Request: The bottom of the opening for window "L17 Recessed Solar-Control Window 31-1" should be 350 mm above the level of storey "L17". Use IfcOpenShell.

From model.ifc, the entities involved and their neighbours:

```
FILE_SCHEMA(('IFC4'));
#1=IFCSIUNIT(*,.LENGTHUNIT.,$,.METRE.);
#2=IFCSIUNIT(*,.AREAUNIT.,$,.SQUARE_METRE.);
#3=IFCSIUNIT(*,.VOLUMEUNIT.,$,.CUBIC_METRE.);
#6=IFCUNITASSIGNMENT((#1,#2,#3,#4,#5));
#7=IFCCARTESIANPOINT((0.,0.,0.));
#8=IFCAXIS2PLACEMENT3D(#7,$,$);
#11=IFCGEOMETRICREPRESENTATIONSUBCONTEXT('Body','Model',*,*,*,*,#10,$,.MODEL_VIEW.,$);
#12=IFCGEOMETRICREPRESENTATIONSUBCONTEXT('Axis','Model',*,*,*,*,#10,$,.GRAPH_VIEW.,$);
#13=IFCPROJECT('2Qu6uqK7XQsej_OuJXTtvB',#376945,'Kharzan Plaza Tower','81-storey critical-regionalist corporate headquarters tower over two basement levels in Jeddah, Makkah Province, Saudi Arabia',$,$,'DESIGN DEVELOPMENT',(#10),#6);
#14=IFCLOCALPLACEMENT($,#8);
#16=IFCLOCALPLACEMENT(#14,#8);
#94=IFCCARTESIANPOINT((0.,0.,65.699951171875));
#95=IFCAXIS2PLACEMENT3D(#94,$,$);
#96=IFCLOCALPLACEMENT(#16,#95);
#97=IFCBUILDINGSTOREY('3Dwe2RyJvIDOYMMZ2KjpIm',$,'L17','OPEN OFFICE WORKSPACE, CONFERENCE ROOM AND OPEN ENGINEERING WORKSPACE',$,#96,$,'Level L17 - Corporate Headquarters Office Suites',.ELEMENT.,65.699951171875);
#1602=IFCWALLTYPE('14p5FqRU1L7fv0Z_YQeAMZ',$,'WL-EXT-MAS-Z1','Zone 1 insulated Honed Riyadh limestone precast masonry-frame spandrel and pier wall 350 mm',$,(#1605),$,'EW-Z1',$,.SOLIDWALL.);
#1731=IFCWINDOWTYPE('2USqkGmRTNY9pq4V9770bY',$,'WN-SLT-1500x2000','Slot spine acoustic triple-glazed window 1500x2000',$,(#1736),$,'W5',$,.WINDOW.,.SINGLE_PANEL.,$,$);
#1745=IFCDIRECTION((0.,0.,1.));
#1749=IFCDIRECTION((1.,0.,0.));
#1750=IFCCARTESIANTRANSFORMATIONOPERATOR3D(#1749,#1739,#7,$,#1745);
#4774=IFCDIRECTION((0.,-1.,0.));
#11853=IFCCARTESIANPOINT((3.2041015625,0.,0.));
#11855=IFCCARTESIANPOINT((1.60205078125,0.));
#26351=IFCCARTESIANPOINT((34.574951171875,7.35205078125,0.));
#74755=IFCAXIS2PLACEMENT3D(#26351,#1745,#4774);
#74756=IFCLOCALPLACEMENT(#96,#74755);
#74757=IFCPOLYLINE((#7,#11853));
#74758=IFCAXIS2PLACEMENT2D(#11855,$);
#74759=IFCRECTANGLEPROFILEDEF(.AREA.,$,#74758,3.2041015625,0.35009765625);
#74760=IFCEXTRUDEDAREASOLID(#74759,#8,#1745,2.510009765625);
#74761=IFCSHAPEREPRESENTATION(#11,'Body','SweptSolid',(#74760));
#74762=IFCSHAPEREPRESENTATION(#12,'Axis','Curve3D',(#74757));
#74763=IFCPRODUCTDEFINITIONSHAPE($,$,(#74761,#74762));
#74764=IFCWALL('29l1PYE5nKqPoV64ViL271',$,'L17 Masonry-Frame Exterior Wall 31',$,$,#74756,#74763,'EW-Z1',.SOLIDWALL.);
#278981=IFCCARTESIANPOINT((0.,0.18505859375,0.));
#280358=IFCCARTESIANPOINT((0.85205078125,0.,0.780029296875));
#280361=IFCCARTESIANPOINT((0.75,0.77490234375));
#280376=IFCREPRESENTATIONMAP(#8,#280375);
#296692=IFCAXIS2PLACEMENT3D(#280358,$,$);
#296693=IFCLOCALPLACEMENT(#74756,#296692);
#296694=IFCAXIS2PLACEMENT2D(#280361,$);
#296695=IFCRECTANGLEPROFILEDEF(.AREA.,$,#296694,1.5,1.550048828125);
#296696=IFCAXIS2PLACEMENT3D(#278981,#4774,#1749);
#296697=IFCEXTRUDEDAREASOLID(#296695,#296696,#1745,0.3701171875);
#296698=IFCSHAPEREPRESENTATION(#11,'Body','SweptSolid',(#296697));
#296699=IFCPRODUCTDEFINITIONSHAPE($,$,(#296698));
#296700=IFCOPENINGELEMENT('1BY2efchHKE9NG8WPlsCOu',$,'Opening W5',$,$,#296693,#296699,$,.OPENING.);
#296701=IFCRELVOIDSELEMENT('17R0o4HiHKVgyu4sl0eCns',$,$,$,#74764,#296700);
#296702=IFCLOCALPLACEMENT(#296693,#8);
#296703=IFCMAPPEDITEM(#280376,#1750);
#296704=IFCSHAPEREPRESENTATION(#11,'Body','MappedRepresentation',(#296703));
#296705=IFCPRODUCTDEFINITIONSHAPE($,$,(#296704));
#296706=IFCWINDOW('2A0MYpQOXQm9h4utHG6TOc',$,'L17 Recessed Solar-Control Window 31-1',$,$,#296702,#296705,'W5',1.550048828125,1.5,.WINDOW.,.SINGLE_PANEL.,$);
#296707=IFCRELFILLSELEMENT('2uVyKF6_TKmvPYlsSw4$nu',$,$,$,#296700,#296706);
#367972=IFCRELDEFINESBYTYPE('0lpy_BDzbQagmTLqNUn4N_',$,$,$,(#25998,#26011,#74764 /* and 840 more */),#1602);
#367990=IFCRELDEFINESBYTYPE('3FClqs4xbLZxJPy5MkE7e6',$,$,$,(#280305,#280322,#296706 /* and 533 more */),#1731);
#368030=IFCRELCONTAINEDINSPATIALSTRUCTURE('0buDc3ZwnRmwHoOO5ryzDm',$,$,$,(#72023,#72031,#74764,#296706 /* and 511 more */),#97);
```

```python
import numpy as np
import ifcopenshell
import ifcopenshell.api.geometry
import ifcopenshell.geom
import ifcopenshell.util.element
import ifcopenshell.util.placement
import ifcopenshell.util.shape
import ifcopenshell.util.unit

model = ifcopenshell.open("model.ifc")
unit_scale = ifcopenshell.util.unit.calculate_unit_scale(model)

window = model.by_id(296706)
opening = window.FillsVoids[0].RelatingOpeningElement
storey = ifcopenshell.util.element.get_container(window, ifc_class="IfcBuildingStorey")
level = ifcopenshell.util.placement.get_local_placement(storey.ObjectPlacement)[2, 3]

# The opening's origin need not be at the sill, so measure its lowest point.
shape = ifcopenshell.geom.create_shape(ifcopenshell.geom.settings(), opening)
bottom = ifcopenshell.util.shape.get_shape_bottom_elevation(shape, shape.geometry) / unit_scale
dz = level + 0.35 / unit_scale - bottom

shift = np.array([0.0, 0.0, dz])
# The window is placed relative to its opening, so it follows when the opening moves.
matrix = ifcopenshell.util.placement.get_local_placement(opening.ObjectPlacement)
matrix[:3, 3] += shift
ifcopenshell.api.geometry.edit_object_placement(
    model, product=opening, matrix=matrix, is_si=False, should_transform_children=True
)

print(f"moved by {dz * unit_scale:+.3f} m")

model.write("model_updated.ifc")
```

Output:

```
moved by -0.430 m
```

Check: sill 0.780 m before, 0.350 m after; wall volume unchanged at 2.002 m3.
